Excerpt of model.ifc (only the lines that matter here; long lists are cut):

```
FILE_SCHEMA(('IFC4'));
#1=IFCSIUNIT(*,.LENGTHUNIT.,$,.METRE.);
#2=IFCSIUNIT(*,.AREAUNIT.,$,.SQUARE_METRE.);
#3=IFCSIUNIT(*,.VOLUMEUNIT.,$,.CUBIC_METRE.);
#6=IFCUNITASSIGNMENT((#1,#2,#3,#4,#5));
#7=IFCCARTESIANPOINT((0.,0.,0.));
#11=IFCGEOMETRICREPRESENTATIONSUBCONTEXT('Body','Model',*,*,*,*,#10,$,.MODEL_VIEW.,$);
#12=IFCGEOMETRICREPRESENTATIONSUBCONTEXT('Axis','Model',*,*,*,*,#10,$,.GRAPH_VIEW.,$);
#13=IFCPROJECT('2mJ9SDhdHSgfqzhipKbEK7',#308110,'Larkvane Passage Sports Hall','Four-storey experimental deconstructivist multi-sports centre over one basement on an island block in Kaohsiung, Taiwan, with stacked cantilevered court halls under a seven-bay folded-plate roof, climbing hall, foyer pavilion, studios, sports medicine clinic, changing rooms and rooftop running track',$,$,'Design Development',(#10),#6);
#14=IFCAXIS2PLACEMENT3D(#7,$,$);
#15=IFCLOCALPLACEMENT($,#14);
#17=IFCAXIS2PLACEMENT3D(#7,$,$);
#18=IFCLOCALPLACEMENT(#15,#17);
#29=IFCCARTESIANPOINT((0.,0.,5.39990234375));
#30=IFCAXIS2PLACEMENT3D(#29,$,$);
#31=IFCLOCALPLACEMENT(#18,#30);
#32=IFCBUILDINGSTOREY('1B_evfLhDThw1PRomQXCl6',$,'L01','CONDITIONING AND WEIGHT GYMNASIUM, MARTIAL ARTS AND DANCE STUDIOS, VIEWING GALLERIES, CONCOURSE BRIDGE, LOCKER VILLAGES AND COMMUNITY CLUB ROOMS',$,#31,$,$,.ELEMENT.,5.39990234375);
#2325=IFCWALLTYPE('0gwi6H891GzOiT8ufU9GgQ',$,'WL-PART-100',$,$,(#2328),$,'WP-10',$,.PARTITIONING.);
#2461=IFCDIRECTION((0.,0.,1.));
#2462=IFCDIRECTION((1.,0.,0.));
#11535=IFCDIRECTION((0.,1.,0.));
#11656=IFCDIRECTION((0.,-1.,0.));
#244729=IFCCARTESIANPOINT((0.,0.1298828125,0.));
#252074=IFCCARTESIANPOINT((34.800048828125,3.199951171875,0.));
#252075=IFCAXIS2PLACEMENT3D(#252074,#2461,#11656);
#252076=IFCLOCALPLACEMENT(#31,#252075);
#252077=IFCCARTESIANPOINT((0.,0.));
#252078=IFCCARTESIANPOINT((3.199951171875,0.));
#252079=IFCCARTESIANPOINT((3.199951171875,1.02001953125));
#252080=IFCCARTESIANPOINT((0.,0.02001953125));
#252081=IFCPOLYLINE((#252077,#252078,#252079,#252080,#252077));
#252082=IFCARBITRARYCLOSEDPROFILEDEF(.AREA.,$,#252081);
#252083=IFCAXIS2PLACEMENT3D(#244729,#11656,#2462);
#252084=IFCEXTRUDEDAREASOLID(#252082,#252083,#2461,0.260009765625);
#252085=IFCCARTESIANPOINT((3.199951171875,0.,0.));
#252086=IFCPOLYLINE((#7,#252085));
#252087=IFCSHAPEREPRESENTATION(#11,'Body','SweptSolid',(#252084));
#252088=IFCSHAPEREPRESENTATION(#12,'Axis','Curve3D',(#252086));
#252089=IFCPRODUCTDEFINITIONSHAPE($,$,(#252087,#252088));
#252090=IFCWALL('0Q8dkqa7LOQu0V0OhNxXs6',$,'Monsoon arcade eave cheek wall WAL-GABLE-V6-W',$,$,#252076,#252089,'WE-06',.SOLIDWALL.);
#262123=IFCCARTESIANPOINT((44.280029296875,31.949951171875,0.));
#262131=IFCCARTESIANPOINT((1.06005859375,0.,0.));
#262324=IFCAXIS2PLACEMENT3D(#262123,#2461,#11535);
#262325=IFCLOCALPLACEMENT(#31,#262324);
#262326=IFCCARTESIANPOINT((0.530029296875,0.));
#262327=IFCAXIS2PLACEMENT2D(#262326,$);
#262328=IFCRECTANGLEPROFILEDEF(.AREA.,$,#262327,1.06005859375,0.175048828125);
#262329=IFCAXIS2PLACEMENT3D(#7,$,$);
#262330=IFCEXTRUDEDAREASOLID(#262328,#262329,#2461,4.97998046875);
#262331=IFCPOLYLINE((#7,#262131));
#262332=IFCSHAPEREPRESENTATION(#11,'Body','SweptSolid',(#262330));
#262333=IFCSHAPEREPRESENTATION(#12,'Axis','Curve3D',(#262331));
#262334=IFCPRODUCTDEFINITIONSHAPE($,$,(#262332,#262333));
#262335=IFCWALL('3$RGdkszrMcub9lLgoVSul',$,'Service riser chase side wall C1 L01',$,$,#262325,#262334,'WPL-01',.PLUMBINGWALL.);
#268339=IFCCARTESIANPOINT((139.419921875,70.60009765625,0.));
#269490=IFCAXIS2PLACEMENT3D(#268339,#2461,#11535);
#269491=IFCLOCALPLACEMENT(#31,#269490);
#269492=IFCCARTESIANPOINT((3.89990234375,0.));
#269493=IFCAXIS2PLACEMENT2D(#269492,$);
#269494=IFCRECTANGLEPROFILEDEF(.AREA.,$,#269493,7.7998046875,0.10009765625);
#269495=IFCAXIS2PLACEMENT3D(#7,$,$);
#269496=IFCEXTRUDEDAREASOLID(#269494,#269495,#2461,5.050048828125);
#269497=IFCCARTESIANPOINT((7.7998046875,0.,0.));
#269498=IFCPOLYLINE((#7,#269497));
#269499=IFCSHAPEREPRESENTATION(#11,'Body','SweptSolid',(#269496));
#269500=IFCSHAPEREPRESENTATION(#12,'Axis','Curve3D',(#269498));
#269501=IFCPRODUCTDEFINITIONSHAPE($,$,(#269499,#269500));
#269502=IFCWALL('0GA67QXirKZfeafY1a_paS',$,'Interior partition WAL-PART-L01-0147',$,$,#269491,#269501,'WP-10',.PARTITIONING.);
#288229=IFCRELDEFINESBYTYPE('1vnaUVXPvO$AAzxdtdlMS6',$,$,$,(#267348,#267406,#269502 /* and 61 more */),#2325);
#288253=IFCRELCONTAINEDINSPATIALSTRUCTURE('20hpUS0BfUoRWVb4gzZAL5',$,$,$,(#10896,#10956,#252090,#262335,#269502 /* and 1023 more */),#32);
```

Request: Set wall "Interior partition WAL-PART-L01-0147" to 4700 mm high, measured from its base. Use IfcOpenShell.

```python
import ifcopenshell
import ifcopenshell.geom
import ifcopenshell.util.representation
import ifcopenshell.util.shape

model = ifcopenshell.open("model.ifc")
settings = ifcopenshell.geom.settings()


def volume(element):
    """Net volume in cubic metres, openings subtracted."""
    shape = ifcopenshell.geom.create_shape(settings, element)
    return ifcopenshell.util.shape.get_volume(shape.geometry)


wall = model.by_guid("0GA67QXirKZfeafY1a_paS")
before = volume(wall)

body = ifcopenshell.util.representation.get_representation(wall, "Model", "Body")
solid = body.Items[0]
old_height = solid.Depth
solid.Depth = 4.7
after = volume(wall)

print(f"height {old_height:g} -> {solid.Depth:g}, volume {before:.3f} -> {after:.3f} m3")

model.write("model_updated.ifc")
```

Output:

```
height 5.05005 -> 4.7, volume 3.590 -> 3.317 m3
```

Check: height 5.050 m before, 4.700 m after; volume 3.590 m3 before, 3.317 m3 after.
